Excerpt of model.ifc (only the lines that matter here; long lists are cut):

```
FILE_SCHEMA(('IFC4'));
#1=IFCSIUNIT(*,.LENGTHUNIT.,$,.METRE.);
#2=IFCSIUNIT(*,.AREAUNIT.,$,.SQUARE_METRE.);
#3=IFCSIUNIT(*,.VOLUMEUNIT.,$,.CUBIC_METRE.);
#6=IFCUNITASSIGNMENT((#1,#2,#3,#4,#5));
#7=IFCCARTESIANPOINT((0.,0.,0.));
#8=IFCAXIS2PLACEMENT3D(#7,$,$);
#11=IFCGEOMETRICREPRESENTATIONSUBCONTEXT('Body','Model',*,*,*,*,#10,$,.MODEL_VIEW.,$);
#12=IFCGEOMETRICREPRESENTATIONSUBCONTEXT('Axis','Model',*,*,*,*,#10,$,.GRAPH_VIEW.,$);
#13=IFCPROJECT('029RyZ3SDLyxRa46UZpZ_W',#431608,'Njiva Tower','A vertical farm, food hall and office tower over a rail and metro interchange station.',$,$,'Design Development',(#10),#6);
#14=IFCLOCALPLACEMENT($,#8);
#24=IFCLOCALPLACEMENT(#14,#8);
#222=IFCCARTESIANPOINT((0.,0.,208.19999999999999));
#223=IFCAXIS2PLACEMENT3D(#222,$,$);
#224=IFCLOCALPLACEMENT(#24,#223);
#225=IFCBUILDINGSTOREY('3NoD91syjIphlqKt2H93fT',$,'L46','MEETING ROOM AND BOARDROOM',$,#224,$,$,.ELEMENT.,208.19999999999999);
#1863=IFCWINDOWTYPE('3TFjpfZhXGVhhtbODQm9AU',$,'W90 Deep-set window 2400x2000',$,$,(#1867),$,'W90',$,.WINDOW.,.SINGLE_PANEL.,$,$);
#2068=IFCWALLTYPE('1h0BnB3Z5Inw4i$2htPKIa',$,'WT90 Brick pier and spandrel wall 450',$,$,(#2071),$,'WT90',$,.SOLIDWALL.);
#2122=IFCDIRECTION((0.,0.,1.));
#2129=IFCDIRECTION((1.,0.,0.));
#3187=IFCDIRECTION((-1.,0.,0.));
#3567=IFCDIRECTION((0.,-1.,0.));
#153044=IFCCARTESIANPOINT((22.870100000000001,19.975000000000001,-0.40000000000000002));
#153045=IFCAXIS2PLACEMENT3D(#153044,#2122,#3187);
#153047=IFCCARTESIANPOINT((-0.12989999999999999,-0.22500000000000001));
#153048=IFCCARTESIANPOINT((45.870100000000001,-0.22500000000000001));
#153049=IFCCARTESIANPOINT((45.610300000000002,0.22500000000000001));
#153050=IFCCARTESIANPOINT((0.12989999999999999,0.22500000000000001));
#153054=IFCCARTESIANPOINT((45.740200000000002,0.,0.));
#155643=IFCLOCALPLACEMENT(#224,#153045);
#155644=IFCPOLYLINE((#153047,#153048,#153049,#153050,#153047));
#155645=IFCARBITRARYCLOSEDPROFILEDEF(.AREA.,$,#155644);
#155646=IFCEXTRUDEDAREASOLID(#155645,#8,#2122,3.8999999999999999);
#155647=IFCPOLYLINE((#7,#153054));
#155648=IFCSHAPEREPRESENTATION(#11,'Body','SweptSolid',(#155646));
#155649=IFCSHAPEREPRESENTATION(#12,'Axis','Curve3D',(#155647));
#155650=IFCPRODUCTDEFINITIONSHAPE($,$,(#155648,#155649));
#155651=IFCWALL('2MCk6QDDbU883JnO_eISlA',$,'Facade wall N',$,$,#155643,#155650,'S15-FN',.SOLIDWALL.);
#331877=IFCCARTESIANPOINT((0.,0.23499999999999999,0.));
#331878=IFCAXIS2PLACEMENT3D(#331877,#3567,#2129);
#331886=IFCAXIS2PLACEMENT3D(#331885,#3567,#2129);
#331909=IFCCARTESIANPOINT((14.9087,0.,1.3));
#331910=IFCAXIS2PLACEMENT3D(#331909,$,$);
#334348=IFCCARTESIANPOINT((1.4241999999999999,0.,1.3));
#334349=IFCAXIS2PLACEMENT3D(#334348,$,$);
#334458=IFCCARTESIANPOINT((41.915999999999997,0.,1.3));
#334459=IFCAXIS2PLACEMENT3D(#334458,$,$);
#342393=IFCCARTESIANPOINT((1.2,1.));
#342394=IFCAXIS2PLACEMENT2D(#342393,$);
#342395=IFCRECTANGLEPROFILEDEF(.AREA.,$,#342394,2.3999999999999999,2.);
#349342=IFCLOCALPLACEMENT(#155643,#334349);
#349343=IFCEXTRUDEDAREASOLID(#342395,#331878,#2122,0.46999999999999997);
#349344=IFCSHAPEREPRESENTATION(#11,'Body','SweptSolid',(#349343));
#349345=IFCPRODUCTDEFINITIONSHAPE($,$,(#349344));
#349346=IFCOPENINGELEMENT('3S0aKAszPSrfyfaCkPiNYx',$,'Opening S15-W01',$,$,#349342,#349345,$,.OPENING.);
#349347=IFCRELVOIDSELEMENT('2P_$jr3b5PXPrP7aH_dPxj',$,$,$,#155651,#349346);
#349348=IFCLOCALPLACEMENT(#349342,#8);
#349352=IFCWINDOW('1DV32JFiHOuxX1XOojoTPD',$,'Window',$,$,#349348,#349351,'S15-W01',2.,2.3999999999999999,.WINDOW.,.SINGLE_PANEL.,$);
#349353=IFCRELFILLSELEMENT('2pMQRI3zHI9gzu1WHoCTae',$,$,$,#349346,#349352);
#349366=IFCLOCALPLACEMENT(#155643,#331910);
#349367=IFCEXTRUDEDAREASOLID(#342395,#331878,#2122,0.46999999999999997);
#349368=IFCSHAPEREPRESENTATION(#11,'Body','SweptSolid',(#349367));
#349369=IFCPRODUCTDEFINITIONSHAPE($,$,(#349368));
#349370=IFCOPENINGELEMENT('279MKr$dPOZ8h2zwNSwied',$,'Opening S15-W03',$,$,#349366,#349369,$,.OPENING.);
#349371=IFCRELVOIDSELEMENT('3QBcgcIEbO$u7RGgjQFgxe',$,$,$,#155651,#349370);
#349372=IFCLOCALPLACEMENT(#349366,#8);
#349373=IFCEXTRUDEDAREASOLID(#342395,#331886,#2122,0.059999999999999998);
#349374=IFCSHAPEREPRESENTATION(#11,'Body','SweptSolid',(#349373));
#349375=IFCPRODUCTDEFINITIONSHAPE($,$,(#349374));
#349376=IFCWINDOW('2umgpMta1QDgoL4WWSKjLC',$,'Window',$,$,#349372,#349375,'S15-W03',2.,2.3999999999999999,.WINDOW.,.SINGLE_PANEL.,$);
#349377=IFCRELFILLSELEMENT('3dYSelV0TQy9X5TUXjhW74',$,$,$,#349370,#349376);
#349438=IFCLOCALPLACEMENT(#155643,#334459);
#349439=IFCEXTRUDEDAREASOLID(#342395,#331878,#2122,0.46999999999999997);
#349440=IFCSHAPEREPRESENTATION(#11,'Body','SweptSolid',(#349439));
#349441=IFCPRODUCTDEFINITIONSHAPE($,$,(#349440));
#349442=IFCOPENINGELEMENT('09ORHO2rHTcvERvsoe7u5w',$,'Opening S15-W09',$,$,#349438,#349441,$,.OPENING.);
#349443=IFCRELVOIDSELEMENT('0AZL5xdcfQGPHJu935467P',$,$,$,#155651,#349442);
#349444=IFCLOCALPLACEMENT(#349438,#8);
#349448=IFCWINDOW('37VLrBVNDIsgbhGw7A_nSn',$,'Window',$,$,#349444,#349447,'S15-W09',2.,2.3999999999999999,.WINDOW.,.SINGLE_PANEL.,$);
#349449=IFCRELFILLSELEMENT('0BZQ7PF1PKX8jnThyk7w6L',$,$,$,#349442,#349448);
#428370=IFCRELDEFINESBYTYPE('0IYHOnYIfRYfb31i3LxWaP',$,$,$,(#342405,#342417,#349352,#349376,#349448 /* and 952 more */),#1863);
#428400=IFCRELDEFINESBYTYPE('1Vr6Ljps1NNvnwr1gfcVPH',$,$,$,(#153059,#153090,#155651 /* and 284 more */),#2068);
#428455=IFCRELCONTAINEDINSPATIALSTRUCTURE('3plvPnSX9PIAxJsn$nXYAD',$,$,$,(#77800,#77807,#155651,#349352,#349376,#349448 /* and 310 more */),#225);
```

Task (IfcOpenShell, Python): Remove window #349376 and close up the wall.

```python
import ifcopenshell
import ifcopenshell.api.feature
import ifcopenshell.api.root
import ifcopenshell.geom
import ifcopenshell.util.shape

model = ifcopenshell.open("model.ifc")
settings = ifcopenshell.geom.settings()


def volume(element):
    """Net volume in cubic metres, openings subtracted."""
    shape = ifcopenshell.geom.create_shape(settings, element)
    return ifcopenshell.util.shape.get_volume(shape.geometry)


window = model.by_id(349376)
opening = window.FillsVoids[0].RelatingOpeningElement
wall = opening.VoidsElements[0].RelatingBuildingElement
before = volume(wall)

ifcopenshell.api.root.remove_product(model, product=window)
ifcopenshell.api.feature.remove_feature(model, feature=opening)

after = volume(wall)

print(f"wall volume {before:.3f} -> {after:.3f} m3")

model.write("model_edited.ifc")
```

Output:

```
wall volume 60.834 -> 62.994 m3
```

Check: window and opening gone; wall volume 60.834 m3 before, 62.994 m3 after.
